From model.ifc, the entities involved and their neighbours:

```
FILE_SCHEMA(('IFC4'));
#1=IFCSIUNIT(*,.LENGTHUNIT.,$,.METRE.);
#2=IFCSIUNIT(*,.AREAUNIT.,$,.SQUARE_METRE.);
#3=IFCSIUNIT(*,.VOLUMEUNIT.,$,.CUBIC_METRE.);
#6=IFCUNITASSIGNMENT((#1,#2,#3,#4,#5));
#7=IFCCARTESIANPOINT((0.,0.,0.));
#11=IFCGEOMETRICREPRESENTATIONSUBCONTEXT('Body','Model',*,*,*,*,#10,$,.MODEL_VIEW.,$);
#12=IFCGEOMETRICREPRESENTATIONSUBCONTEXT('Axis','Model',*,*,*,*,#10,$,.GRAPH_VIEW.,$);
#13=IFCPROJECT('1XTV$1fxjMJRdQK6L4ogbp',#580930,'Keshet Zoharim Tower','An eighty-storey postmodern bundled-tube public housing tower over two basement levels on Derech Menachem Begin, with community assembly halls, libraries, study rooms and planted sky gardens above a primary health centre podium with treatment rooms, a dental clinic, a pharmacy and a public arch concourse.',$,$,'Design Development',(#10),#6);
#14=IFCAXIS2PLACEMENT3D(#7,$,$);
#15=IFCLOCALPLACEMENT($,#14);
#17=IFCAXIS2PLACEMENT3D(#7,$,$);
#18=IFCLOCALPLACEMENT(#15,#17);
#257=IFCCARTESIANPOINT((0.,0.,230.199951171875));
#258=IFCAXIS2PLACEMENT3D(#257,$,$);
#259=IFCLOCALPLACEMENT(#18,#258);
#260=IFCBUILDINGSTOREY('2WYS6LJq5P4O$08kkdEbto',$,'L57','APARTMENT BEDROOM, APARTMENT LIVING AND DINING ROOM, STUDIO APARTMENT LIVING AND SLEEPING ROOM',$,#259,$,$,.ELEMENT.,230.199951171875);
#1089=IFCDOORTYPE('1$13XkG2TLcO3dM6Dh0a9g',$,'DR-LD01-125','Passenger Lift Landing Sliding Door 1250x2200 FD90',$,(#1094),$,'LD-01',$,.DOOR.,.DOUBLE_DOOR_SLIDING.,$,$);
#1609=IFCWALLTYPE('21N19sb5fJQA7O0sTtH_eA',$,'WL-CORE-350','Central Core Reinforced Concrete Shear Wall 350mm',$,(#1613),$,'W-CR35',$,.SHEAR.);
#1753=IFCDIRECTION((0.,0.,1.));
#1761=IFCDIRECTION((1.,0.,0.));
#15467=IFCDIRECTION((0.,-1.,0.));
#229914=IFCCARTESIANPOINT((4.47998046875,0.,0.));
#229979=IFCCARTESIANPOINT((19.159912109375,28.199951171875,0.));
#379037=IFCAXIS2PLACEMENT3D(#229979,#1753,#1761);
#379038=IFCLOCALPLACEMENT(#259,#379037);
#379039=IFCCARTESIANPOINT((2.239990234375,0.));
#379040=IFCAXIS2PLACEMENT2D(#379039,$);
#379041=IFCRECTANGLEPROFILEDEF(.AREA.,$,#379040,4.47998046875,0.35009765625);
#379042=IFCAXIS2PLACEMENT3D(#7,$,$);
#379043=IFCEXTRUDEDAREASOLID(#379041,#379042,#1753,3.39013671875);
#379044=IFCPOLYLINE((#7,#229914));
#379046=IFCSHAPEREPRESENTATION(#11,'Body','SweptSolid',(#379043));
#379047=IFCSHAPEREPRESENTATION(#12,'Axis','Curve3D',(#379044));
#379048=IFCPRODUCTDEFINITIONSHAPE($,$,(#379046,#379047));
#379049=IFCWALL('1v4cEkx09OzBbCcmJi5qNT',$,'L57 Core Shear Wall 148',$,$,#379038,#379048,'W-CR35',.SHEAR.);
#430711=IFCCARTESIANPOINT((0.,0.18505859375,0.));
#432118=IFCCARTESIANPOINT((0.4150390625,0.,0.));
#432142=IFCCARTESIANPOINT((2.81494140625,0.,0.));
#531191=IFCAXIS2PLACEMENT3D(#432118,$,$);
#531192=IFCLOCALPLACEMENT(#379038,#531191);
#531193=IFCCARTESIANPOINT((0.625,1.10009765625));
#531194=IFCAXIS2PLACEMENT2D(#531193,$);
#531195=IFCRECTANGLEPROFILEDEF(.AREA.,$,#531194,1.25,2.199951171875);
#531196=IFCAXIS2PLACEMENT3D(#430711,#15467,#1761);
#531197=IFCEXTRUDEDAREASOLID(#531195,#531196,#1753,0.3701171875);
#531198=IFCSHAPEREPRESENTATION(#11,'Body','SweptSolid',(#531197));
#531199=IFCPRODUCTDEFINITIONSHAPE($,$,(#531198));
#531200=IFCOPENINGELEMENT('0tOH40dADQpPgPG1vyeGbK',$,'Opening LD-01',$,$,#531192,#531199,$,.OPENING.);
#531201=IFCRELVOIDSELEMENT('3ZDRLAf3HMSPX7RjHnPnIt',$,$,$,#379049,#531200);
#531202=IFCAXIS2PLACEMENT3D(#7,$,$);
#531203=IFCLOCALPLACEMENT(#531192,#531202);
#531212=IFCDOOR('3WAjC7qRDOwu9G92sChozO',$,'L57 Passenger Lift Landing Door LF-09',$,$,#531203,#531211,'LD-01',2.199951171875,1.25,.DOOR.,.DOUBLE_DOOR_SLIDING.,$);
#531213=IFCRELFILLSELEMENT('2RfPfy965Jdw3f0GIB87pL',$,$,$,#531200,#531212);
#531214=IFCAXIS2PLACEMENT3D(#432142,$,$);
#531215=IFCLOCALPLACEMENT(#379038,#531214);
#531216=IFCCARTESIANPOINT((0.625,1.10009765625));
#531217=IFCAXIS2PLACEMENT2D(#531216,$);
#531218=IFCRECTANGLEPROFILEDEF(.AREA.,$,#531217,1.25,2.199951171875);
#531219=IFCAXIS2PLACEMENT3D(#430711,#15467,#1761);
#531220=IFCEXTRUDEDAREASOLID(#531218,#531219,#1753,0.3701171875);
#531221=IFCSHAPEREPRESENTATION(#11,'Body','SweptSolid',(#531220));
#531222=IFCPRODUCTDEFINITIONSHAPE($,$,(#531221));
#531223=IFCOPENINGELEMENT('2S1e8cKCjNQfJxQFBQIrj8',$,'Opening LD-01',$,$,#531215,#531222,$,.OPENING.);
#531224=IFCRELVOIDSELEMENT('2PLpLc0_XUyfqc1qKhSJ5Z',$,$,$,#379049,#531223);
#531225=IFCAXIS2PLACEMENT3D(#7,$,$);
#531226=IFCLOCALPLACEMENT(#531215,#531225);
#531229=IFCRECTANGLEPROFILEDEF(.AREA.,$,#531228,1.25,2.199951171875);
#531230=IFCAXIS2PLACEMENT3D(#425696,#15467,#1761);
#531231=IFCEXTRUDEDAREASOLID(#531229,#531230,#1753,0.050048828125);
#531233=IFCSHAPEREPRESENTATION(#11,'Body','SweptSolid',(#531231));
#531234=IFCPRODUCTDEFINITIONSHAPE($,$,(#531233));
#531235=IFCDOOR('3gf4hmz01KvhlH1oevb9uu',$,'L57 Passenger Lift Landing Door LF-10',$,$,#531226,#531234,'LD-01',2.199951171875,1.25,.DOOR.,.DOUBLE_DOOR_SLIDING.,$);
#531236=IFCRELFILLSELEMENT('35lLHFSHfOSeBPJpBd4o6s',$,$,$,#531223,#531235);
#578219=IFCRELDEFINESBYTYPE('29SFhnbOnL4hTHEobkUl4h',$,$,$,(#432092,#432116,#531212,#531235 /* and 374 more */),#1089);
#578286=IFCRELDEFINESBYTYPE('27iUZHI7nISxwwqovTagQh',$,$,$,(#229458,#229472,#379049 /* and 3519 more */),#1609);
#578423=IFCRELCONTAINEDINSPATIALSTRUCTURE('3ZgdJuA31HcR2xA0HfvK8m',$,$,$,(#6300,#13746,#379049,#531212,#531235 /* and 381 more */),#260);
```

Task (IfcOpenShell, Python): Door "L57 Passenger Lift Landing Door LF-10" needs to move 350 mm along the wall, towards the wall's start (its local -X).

```python
import ifcopenshell
import ifcopenshell.api.geometry
import ifcopenshell.util.placement

model = ifcopenshell.open("model.ifc")

door = model.by_guid("3gf4hmz01KvhlH1oevb9uu")
opening = door.FillsVoids[0].RelatingOpeningElement
wall = opening.VoidsElements[0].RelatingBuildingElement

wall_matrix = ifcopenshell.util.placement.get_local_placement(wall.ObjectPlacement)
shift = wall_matrix[:3, 0] * -0.35
before = ifcopenshell.util.placement.get_local_placement(door.ObjectPlacement)[:3, 3].copy()

# The door is placed relative to its opening, so it follows when the opening moves.
matrix = ifcopenshell.util.placement.get_local_placement(opening.ObjectPlacement)
matrix[:3, 3] += shift
ifcopenshell.api.geometry.edit_object_placement(
    model, product=opening, matrix=matrix, is_si=False, should_transform_children=True
)

after = ifcopenshell.util.placement.get_local_placement(door.ObjectPlacement)[:3, 3]
print("door moved by", (after - before).round(3) + 0.0)

model.write("model-out.ifc")
```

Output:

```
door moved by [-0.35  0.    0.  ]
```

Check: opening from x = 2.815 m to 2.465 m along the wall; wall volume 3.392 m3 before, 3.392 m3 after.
